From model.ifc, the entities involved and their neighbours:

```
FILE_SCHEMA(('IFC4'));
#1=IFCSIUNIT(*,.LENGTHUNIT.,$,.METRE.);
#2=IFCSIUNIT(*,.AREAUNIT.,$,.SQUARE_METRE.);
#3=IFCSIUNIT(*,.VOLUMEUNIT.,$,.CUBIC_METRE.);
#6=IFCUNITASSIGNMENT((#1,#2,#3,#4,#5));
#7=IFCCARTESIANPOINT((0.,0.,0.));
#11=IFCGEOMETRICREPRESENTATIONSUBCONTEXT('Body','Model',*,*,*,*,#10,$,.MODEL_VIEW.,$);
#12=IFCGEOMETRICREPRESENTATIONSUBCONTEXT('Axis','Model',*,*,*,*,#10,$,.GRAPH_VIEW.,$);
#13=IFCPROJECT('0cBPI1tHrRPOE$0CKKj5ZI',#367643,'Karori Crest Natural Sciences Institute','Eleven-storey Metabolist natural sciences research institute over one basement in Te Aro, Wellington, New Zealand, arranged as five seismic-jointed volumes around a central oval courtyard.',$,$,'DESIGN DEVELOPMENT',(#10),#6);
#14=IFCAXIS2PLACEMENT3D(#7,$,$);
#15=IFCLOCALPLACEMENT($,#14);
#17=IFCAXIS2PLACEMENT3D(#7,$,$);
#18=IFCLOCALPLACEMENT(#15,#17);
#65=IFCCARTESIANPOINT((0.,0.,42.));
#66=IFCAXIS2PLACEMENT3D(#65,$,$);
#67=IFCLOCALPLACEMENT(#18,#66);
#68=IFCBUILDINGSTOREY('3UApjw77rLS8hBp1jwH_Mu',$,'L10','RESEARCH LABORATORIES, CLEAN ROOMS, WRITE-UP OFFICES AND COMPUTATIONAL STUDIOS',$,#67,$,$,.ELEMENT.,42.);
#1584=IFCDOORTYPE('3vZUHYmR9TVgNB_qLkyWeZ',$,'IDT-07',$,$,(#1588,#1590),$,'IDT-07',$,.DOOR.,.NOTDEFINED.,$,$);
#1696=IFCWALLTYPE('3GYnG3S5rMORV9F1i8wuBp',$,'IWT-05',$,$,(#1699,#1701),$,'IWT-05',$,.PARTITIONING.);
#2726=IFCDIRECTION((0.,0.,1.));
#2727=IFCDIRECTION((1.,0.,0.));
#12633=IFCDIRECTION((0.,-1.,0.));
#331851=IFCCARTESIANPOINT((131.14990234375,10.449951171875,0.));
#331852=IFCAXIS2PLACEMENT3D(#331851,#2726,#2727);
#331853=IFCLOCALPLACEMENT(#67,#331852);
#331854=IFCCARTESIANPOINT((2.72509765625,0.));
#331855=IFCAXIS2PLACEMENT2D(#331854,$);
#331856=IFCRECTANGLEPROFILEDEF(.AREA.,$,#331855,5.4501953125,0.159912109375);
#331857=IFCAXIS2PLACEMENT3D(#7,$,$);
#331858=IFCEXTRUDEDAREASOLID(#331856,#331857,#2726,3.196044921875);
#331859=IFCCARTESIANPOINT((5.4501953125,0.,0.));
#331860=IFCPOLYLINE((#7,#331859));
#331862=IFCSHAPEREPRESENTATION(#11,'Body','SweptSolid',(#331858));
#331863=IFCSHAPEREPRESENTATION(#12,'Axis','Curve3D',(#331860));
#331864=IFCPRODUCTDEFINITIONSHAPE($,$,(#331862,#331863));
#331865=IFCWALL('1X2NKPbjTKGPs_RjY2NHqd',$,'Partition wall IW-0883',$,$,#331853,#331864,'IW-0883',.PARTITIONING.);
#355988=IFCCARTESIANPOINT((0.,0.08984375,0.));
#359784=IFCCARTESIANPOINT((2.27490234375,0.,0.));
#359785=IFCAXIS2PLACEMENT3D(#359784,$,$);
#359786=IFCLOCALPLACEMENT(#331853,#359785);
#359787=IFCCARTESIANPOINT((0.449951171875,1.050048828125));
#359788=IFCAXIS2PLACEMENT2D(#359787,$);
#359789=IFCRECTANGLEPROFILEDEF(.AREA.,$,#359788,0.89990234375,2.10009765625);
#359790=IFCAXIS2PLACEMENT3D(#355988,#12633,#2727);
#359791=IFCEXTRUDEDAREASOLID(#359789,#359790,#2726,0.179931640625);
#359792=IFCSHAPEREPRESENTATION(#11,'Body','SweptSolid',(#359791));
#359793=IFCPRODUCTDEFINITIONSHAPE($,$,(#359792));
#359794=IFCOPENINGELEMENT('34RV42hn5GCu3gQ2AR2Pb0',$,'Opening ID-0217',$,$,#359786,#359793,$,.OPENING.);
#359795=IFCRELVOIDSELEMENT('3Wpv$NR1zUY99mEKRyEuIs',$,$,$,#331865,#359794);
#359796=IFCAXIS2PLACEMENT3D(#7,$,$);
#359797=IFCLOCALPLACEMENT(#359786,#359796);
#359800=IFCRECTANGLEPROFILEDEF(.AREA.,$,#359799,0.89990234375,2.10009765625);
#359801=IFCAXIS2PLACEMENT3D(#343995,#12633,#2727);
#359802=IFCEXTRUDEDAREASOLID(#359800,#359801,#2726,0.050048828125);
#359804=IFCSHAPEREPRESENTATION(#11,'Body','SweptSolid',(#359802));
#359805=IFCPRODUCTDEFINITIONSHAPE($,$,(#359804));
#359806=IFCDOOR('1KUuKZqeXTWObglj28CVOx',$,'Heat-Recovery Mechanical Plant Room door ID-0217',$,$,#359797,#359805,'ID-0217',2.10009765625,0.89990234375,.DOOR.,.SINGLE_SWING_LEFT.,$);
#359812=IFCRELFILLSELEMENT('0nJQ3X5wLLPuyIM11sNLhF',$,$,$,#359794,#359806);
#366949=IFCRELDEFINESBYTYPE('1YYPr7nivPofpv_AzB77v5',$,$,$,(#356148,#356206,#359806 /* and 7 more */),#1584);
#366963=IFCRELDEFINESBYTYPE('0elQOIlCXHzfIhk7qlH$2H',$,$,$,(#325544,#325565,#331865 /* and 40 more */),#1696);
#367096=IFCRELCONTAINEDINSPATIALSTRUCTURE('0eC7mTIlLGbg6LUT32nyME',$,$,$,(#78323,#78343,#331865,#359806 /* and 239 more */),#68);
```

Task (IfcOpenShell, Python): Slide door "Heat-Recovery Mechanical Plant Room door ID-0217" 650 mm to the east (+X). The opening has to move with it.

```python
import ifcopenshell
import ifcopenshell.api.geometry
import ifcopenshell.util.placement
import ifcopenshell.util.unit

model = ifcopenshell.open("model.ifc")
unit_scale = ifcopenshell.util.unit.calculate_unit_scale(model)

door = model.by_guid("1KUuKZqeXTWObglj28CVOx")
opening = door.FillsVoids[0].RelatingOpeningElement
wall = opening.VoidsElements[0].RelatingBuildingElement

wall_matrix = ifcopenshell.util.placement.get_local_placement(wall.ObjectPlacement)
shift = wall_matrix[:3, 0] * 0.65 / unit_scale
before = ifcopenshell.util.placement.get_local_placement(door.ObjectPlacement)[:3, 3].copy()

# The door is placed relative to its opening, so it follows when the opening moves.
matrix = ifcopenshell.util.placement.get_local_placement(opening.ObjectPlacement)
matrix[:3, 3] += shift
ifcopenshell.api.geometry.edit_object_placement(
    model, product=opening, matrix=matrix, is_si=False, should_transform_children=True
)

after = ifcopenshell.util.placement.get_local_placement(door.ObjectPlacement)[:3, 3]
print("door moved by", (after - before).round(3) + 0.0)

model.write("model-out.ifc")
```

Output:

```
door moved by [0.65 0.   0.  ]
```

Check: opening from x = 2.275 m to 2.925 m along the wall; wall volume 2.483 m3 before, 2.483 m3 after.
